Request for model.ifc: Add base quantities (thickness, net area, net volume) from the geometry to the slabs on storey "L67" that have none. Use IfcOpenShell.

First a look at what the model holds.

```python
import ifcopenshell
import ifcopenshell.util.element
import ifcopenshell.util.unit

model = ifcopenshell.open("model.ifc")
print(model.schema)
for unit_type in ("LENGTHUNIT", "AREAUNIT", "VOLUMEUNIT"):
    print(unit_type, ifcopenshell.util.unit.calculate_unit_scale(model, unit_type))
storey = next(s for s in model.by_type("IfcBuildingStorey") if s.Name == "L67")
slabs = [e for e in ifcopenshell.util.element.get_decomposition(storey) if e.is_a("IfcSlab")]
for e in sorted(slabs, key=lambda e: e.id()):
    print(e.id(), e.is_a(), e.Name, list(ifcopenshell.util.element.get_psets(e, qtos_only=True)), sep=" | ")
```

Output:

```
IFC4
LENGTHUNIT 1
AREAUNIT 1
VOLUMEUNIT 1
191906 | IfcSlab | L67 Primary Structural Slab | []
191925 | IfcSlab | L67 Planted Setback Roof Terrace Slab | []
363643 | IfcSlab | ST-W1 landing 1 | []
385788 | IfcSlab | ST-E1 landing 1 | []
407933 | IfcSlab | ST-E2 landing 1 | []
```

```python
import ifcopenshell
import ifcopenshell.api.pset
import ifcopenshell.geom
import ifcopenshell.util.element
import ifcopenshell.util.shape
import ifcopenshell.util.unit

model = ifcopenshell.open("model.ifc")
unit_scale = ifcopenshell.util.unit.calculate_unit_scale(model)
area_scale = ifcopenshell.util.unit.calculate_unit_scale(model, "AREAUNIT")
volume_scale = ifcopenshell.util.unit.calculate_unit_scale(model, "VOLUMEUNIT")
settings = ifcopenshell.geom.settings()

storey = next(s for s in model.by_type("IfcBuildingStorey") if s.Name == "L67")
slabs = [e for e in ifcopenshell.util.element.get_decomposition(storey) if e.is_a("IfcSlab")]

for e in sorted(slabs, key=lambda e: e.id()):
    if ifcopenshell.util.element.get_psets(e, qtos_only=True, should_inherit=False):
        continue
    # Geometry comes back in metres, in the element's own axes.
    shape = ifcopenshell.geom.create_shape(settings, e)
    values = {
        "Width": ifcopenshell.util.shape.get_z(shape.geometry) / unit_scale,
        "NetArea": ifcopenshell.util.shape.get_footprint_area(shape.geometry) / area_scale,
        "NetVolume": ifcopenshell.util.shape.get_volume(shape.geometry) / volume_scale,
    }
    qto = ifcopenshell.api.pset.add_qto(model, product=e, name="Qto_SlabBaseQuantities")
    ifcopenshell.api.pset.edit_qto(model, qto=qto, properties=values)
    print(e.id(), {k: round(v, 3) for k, v in values.items()})

model.write("model_rev.ifc")
```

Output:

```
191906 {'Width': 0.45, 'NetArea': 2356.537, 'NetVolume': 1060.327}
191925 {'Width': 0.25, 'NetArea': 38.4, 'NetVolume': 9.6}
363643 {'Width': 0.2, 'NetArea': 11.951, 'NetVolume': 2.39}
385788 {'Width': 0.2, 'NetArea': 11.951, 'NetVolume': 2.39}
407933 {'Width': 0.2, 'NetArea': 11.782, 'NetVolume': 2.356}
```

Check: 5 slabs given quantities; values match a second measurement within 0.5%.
